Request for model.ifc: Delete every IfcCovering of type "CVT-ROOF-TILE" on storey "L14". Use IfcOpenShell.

First a look at what the model holds.

```python
import ifcopenshell
import ifcopenshell.util.element

model = ifcopenshell.open("model.ifc")
print(model.schema)
storey = next(s for s in model.by_type("IfcBuildingStorey") if s.Name == "L14")
coverings = [e for e in ifcopenshell.util.element.get_decomposition(storey) if e.is_a("IfcCovering")]
seen = {}
for e in coverings:
    element_type = ifcopenshell.util.element.get_type(e)
    name = element_type.Name if element_type not in (None, e) else None
    seen[name] = seen.get(name, 0) + 1
for name, count in sorted(seen.items(), key=str):
    print(count, "x", name)
```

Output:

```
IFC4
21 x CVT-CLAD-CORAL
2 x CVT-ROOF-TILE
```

```python
import ifcopenshell
import ifcopenshell.api.root
import ifcopenshell.util.element

model = ifcopenshell.open("model.ifc")

storey = next(s for s in model.by_type("IfcBuildingStorey") if s.Name == "L14")
coverings = [e for e in ifcopenshell.util.element.get_decomposition(storey) if e.is_a("IfcCovering")]
targets = [e for e in coverings if (t := ifcopenshell.util.element.get_type(e)) not in (None, e) and t.Name == "CVT-ROOF-TILE"]

for e in targets:
    ifcopenshell.api.root.remove_product(model, product=e)
print(len(targets), "removed")

model.write("model_rev.ifc")
```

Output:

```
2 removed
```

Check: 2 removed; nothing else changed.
